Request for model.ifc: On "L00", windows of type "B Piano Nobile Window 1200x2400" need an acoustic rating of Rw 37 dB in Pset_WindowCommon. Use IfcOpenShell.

First a look at what the model holds.

```python
import ifcopenshell
import ifcopenshell.util.element

model = ifcopenshell.open("model.ifc")
print(model.schema)
storey = next(s for s in model.by_type("IfcBuildingStorey") if s.Name == "L00")
windows = [e for e in ifcopenshell.util.element.get_decomposition(storey) if e.is_a("IfcWindow")]
seen = {}
for e in windows:
    element_type = ifcopenshell.util.element.get_type(e)
    key = (element_type.Name if element_type != e and element_type else None, ifcopenshell.util.element.get_pset(e, "Pset_WindowCommon", "AcousticRating"))
    seen[key] = seen.get(key, 0) + 1
for (name, value), count in sorted(seen.items(), key=str):
    print(count, "x", name, "|", value)
```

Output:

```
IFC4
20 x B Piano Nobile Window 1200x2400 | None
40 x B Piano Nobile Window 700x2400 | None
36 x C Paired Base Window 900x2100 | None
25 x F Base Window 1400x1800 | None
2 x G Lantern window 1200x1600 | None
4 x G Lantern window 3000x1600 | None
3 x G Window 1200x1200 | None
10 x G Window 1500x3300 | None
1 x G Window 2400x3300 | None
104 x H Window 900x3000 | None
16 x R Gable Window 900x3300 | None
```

```python
import ifcopenshell
import ifcopenshell.api.pset
import ifcopenshell.util.element

model = ifcopenshell.open("model.ifc")

storey = next(s for s in model.by_type("IfcBuildingStorey") if s.Name == "L00")
windows = [e for e in ifcopenshell.util.element.get_decomposition(storey) if e.is_a("IfcWindow")]

count = 0
for e in windows:
    element_type = ifcopenshell.util.element.get_type(e)
    if element_type in (None, e) or element_type.Name != "B Piano Nobile Window 1200x2400":
        continue
    # add_pset returns the element's existing set when there is one.
    pset = ifcopenshell.api.pset.add_pset(model, product=e, name="Pset_WindowCommon")
    ifcopenshell.api.pset.edit_pset(model, pset=pset, properties={"AcousticRating": "Rw 37 dB"})
    count += 1

print(count, "windows updated")

model.write("model_updated.ifc")
```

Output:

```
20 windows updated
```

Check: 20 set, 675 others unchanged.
